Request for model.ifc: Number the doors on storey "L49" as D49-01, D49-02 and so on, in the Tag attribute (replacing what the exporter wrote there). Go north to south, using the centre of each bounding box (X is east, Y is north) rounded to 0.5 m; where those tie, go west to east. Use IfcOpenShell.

First a look at what the model holds.

```python
import ifcopenshell
import ifcopenshell.util.element
import ifcopenshell.util.placement

model = ifcopenshell.open("model.ifc")
print(model.schema)
storey = next(s for s in model.by_type("IfcBuildingStorey") if s.Name == "L49")
doors = [e for e in ifcopenshell.util.element.get_decomposition(storey) if e.is_a("IfcDoor")]
for e in sorted(doors, key=lambda e: e.id()):
    origin = ifcopenshell.util.placement.get_local_placement(e.ObjectPlacement)[:3, 3]
    print(e.id(), e.Tag, e.Name, origin.round(2) + 0.0, sep=" | ")
```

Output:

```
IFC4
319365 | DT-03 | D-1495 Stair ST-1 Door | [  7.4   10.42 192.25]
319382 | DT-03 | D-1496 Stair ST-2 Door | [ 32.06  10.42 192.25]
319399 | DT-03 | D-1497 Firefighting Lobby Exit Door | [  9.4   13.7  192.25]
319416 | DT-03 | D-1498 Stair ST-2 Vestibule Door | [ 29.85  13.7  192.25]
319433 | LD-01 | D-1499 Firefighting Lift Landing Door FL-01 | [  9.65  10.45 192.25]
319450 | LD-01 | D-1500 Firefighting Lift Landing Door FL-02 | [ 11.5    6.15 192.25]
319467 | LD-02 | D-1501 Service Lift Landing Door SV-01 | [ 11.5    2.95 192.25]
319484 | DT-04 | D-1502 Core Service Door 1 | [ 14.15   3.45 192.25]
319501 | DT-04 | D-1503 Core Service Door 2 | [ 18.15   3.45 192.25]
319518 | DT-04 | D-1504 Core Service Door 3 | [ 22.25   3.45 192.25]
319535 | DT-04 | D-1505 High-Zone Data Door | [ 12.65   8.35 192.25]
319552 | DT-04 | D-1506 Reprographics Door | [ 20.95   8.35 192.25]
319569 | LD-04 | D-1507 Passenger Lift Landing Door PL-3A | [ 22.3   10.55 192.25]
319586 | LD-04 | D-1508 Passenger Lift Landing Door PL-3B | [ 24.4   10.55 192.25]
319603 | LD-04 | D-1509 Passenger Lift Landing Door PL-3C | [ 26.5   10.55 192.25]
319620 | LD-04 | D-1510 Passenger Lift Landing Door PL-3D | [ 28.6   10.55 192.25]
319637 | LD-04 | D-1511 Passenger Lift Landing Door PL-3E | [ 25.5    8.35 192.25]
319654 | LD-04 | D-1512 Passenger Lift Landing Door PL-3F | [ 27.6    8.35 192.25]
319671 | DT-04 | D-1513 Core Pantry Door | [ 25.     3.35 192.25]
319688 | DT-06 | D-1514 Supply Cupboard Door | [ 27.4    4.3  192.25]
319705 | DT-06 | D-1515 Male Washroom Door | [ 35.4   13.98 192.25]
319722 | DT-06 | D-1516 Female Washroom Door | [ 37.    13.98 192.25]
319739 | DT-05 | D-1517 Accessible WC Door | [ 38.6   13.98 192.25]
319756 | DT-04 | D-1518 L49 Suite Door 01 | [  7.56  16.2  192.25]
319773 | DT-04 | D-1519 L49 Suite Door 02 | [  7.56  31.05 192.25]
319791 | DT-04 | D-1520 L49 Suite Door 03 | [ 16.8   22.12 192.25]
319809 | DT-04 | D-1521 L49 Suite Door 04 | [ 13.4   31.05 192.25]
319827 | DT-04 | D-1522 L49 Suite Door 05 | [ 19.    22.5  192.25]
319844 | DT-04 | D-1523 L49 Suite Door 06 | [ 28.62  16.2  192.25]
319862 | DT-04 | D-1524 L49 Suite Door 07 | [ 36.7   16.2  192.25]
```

```python
import ifcopenshell
import ifcopenshell.geom
import ifcopenshell.util.element
import ifcopenshell.util.shape

model = ifcopenshell.open("model.ifc")
settings = ifcopenshell.geom.settings()
settings.set("use-world-coords", True)


def centre(element):
    shape = ifcopenshell.geom.create_shape(settings, element)
    return ifcopenshell.util.shape.get_bbox_centroid(shape.geometry)


storey = next(s for s in model.by_type("IfcBuildingStorey") if s.Name == "L49")
doors = [e for e in ifcopenshell.util.element.get_decomposition(storey) if e.is_a("IfcDoor")]

# Insertion points can sit at a corner or the storey origin, so sort by the geometry (in metres).
centres = {e: centre(e) for e in doors}
doors.sort(key=lambda e: (-round(centres[e][1] / 0.5), centres[e][0]))

for i, e in enumerate(doors, start=1):
    number = f"D49-{i:02d}"
    e.Tag = number
    print(e.id(), number)

model.write("model_updated.ifc")
```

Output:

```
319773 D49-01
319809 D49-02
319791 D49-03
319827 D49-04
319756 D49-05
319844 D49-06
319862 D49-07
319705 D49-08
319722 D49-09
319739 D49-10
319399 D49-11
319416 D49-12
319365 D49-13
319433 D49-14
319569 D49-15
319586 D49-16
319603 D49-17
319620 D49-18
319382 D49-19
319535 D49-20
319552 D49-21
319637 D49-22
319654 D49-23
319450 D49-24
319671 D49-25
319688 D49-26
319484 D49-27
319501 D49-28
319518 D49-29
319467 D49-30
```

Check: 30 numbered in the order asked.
